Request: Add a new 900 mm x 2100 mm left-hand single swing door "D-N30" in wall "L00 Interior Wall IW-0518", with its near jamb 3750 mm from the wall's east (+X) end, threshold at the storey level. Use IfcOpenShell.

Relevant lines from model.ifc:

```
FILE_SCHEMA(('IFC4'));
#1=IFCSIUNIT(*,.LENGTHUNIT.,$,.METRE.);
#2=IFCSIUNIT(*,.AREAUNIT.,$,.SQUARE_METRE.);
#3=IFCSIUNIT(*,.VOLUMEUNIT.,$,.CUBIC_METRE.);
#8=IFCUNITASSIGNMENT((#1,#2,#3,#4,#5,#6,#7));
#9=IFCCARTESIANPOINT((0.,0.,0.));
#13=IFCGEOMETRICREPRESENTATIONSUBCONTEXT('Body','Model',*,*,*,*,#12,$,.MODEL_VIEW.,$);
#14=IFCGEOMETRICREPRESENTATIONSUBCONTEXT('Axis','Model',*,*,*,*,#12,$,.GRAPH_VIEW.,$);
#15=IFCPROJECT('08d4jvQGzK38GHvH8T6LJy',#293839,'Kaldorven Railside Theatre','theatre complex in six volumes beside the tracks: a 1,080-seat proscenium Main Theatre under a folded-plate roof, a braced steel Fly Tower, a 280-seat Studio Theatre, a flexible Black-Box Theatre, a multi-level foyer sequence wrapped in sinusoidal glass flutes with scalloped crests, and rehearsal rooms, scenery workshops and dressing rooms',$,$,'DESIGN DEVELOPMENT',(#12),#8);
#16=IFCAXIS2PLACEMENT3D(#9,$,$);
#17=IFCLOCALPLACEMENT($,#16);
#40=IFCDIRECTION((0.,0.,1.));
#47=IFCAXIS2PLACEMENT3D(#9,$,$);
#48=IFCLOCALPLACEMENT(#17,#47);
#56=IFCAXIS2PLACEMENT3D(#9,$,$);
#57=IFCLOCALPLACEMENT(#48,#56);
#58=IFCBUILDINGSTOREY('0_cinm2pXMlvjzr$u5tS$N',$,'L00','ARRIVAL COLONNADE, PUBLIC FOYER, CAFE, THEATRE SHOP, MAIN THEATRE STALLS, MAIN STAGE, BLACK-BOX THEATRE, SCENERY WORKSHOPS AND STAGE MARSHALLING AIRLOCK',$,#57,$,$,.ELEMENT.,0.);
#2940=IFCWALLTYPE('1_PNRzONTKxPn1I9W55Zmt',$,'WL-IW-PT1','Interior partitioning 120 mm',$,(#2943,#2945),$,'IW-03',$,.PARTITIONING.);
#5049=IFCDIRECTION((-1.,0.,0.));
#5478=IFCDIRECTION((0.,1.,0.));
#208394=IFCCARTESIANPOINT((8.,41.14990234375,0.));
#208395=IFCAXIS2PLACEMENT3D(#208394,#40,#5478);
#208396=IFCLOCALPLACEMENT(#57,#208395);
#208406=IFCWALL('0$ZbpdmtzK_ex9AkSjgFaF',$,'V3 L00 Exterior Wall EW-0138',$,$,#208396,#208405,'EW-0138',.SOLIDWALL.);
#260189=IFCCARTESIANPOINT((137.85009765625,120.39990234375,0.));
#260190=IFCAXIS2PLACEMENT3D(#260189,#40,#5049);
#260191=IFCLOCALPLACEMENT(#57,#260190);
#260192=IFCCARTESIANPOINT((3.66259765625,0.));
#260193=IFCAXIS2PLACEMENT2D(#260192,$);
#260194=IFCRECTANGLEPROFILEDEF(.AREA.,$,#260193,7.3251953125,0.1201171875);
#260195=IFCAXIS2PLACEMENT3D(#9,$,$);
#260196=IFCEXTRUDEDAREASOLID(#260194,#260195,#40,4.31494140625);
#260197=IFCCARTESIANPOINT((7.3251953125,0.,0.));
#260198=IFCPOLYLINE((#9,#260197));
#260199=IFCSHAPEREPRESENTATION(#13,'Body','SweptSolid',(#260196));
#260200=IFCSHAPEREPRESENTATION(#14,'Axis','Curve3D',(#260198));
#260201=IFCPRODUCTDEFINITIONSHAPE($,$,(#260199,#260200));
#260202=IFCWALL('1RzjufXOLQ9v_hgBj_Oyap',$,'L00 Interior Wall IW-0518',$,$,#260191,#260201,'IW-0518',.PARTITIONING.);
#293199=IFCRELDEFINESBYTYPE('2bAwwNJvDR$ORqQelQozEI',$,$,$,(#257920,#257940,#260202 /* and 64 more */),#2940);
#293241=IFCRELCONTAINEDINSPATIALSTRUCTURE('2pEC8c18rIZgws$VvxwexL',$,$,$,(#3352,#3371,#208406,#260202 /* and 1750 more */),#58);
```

```python
import numpy as np
import ifcopenshell
import ifcopenshell.api.feature
import ifcopenshell.api.geometry
import ifcopenshell.api.root
import ifcopenshell.api.spatial
import ifcopenshell.geom
import ifcopenshell.util.element
import ifcopenshell.util.placement
import ifcopenshell.util.representation
import ifcopenshell.util.shape
import ifcopenshell.util.unit

model = ifcopenshell.open("model.ifc")
unit_scale = ifcopenshell.util.unit.calculate_unit_scale(model)
settings = ifcopenshell.geom.settings()


def volume(element):
    """Net volume in cubic metres, openings subtracted."""
    shape = ifcopenshell.geom.create_shape(settings, element)
    return ifcopenshell.util.shape.get_volume(shape.geometry)


wall = model.by_guid("1RzjufXOLQ9v_hgBj_Oyap")
storey = ifcopenshell.util.element.get_container(wall, ifc_class="IfcBuildingStorey")
context = ifcopenshell.util.representation.get_context(model, "Model", "Body", "MODEL_VIEW")
before = volume(wall)

width, height, from_end, sill = 0.9, 2.1, 3.75, 0.0  # metres

# The wall runs along its own X axis, and the end named is its -X end.
wall_shape = ifcopenshell.geom.create_shape(settings, wall)
x, y, z = ifcopenshell.util.shape.get_vertices(wall_shape.geometry).T
start = x.min() + from_end
face, thickness = float(y.min()), float(y.max() - y.min())
wall_matrix = ifcopenshell.util.placement.get_local_placement(wall.ObjectPlacement)
level = ifcopenshell.util.placement.get_local_placement(storey.ObjectPlacement)[2, 3]


def in_wall(x, y):
    """Placement at x, y metres in the wall's axes, at sill height."""
    matrix = wall_matrix.copy()
    matrix[:, 3] = wall_matrix @ np.array([x / unit_scale, y / unit_scale, 0.0, 1.0])
    matrix[2, 3] = level + sill / unit_scale
    return matrix


# Opening: a box that overshoots both wall faces by 50 mm.
opening = ifcopenshell.api.root.create_entity(model, ifc_class="IfcOpeningElement", predefined_type="OPENING")
box = ifcopenshell.api.geometry.add_wall_representation(
    model, context=context, length=width, height=height, thickness=thickness + 0.1
)
ifcopenshell.api.geometry.assign_representation(model, product=opening, representation=box)
ifcopenshell.api.geometry.edit_object_placement(model, product=opening, matrix=in_wall(start, face - 0.05), is_si=False)
ifcopenshell.api.feature.add_feature(model, feature=opening, element=wall)

door = ifcopenshell.api.root.create_entity(model, ifc_class="IfcDoor", name="D-N30", predefined_type="DOOR")
door.OverallWidth, door.OverallHeight = width / unit_scale, height / unit_scale
door.OperationType = "SINGLE_SWING_LEFT"
body = ifcopenshell.api.geometry.add_door_representation(
    model,
    context=context,
    overall_width=door.OverallWidth,
    overall_height=door.OverallHeight,
    operation_type="SINGLE_SWING_LEFT",
    lining_properties={"LiningDepth": thickness / unit_scale, "ThresholdDepth": thickness / unit_scale},
)
ifcopenshell.api.geometry.assign_representation(model, product=door, representation=body)
ifcopenshell.api.spatial.assign_container(model, products=[door], relating_structure=storey)
ifcopenshell.api.feature.add_filling(model, opening=opening, element=door)

# The lining spans the wall, so the door starts at the wall face.
ifcopenshell.api.geometry.edit_object_placement(model, product=door, matrix=in_wall(start, face), is_si=False)

after = volume(wall)

print(f"wall volume {before:.3f} -> {after:.3f} m3")

model.write("model_edited.ifc")
```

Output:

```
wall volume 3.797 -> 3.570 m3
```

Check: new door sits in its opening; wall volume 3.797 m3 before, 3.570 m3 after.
